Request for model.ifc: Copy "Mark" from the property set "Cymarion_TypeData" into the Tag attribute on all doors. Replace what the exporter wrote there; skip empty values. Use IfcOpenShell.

First a look at what the model holds.

```python
import ifcopenshell
import ifcopenshell.util.element

model = ifcopenshell.open("model.ifc")
print(model.schema)
doors = model.by_type("IfcDoor")
print(len(doors), "doors")
for e in doors[:8]:
    source = ifcopenshell.util.element.get_pset(e, "Cymarion_TypeData", "Mark")
    target = e.Tag
    print(e.id(), repr(source), repr(target), sep=" | ")
```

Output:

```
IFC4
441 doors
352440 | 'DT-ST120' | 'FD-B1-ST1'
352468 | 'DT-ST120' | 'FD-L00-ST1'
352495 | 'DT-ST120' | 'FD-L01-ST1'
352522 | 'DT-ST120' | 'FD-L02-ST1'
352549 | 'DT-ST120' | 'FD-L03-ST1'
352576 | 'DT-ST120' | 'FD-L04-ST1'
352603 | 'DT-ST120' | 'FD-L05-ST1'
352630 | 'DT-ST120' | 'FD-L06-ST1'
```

```python
import ifcopenshell
import ifcopenshell.util.element

model = ifcopenshell.open("model.ifc")

count = 0
for e in model.by_type("IfcDoor"):
    value = ifcopenshell.util.element.get_pset(e, "Cymarion_TypeData", "Mark")
    current = e.Tag
    if not value or not value.strip() or current == value:
        continue
    e.Tag = value
    count += 1

print(count, "doors updated")

model.write("model_rev.ifc")
```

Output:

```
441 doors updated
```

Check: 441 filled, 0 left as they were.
